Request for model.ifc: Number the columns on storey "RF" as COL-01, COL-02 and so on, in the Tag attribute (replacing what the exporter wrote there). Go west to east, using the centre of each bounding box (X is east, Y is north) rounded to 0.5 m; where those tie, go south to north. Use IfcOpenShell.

First a look at what the model holds.

```python
import ifcopenshell
import ifcopenshell.util.element
import ifcopenshell.util.placement

model = ifcopenshell.open("model.ifc")
print(model.schema)
storey = next(s for s in model.by_type("IfcBuildingStorey") if s.Name == "RF")
columns = [e for e in ifcopenshell.util.element.get_decomposition(storey) if e.is_a("IfcColumn")]
for e in sorted(columns, key=lambda e: e.id()):
    origin = ifcopenshell.util.placement.get_local_placement(e.ObjectPlacement)[:3, 3]
    print(e.id(), e.Tag, e.Name, origin.round(2) + 0.0, sep=" | ")
```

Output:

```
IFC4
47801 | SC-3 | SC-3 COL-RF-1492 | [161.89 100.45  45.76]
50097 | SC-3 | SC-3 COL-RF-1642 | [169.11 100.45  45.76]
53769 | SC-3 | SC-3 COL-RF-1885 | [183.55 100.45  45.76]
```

```python
import ifcopenshell
import ifcopenshell.geom
import ifcopenshell.util.element
import ifcopenshell.util.shape

model = ifcopenshell.open("model.ifc")
settings = ifcopenshell.geom.settings()
settings.set("use-world-coords", True)


def centre(element):
    shape = ifcopenshell.geom.create_shape(settings, element)
    return ifcopenshell.util.shape.get_bbox_centroid(shape.geometry)


storey = next(s for s in model.by_type("IfcBuildingStorey") if s.Name == "RF")
columns = [e for e in ifcopenshell.util.element.get_decomposition(storey) if e.is_a("IfcColumn")]

# Insertion points can sit at a corner or the storey origin, so sort by the geometry (in metres).
centres = {e: centre(e) for e in columns}
columns.sort(key=lambda e: (round(centres[e][0] / 0.5), centres[e][1]))

for i, e in enumerate(columns, start=1):
    number = f"COL-{i:02d}"
    e.Tag = number
    print(e.id(), number)

model.write("model_updated.ifc")
```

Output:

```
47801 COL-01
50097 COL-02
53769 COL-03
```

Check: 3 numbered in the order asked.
